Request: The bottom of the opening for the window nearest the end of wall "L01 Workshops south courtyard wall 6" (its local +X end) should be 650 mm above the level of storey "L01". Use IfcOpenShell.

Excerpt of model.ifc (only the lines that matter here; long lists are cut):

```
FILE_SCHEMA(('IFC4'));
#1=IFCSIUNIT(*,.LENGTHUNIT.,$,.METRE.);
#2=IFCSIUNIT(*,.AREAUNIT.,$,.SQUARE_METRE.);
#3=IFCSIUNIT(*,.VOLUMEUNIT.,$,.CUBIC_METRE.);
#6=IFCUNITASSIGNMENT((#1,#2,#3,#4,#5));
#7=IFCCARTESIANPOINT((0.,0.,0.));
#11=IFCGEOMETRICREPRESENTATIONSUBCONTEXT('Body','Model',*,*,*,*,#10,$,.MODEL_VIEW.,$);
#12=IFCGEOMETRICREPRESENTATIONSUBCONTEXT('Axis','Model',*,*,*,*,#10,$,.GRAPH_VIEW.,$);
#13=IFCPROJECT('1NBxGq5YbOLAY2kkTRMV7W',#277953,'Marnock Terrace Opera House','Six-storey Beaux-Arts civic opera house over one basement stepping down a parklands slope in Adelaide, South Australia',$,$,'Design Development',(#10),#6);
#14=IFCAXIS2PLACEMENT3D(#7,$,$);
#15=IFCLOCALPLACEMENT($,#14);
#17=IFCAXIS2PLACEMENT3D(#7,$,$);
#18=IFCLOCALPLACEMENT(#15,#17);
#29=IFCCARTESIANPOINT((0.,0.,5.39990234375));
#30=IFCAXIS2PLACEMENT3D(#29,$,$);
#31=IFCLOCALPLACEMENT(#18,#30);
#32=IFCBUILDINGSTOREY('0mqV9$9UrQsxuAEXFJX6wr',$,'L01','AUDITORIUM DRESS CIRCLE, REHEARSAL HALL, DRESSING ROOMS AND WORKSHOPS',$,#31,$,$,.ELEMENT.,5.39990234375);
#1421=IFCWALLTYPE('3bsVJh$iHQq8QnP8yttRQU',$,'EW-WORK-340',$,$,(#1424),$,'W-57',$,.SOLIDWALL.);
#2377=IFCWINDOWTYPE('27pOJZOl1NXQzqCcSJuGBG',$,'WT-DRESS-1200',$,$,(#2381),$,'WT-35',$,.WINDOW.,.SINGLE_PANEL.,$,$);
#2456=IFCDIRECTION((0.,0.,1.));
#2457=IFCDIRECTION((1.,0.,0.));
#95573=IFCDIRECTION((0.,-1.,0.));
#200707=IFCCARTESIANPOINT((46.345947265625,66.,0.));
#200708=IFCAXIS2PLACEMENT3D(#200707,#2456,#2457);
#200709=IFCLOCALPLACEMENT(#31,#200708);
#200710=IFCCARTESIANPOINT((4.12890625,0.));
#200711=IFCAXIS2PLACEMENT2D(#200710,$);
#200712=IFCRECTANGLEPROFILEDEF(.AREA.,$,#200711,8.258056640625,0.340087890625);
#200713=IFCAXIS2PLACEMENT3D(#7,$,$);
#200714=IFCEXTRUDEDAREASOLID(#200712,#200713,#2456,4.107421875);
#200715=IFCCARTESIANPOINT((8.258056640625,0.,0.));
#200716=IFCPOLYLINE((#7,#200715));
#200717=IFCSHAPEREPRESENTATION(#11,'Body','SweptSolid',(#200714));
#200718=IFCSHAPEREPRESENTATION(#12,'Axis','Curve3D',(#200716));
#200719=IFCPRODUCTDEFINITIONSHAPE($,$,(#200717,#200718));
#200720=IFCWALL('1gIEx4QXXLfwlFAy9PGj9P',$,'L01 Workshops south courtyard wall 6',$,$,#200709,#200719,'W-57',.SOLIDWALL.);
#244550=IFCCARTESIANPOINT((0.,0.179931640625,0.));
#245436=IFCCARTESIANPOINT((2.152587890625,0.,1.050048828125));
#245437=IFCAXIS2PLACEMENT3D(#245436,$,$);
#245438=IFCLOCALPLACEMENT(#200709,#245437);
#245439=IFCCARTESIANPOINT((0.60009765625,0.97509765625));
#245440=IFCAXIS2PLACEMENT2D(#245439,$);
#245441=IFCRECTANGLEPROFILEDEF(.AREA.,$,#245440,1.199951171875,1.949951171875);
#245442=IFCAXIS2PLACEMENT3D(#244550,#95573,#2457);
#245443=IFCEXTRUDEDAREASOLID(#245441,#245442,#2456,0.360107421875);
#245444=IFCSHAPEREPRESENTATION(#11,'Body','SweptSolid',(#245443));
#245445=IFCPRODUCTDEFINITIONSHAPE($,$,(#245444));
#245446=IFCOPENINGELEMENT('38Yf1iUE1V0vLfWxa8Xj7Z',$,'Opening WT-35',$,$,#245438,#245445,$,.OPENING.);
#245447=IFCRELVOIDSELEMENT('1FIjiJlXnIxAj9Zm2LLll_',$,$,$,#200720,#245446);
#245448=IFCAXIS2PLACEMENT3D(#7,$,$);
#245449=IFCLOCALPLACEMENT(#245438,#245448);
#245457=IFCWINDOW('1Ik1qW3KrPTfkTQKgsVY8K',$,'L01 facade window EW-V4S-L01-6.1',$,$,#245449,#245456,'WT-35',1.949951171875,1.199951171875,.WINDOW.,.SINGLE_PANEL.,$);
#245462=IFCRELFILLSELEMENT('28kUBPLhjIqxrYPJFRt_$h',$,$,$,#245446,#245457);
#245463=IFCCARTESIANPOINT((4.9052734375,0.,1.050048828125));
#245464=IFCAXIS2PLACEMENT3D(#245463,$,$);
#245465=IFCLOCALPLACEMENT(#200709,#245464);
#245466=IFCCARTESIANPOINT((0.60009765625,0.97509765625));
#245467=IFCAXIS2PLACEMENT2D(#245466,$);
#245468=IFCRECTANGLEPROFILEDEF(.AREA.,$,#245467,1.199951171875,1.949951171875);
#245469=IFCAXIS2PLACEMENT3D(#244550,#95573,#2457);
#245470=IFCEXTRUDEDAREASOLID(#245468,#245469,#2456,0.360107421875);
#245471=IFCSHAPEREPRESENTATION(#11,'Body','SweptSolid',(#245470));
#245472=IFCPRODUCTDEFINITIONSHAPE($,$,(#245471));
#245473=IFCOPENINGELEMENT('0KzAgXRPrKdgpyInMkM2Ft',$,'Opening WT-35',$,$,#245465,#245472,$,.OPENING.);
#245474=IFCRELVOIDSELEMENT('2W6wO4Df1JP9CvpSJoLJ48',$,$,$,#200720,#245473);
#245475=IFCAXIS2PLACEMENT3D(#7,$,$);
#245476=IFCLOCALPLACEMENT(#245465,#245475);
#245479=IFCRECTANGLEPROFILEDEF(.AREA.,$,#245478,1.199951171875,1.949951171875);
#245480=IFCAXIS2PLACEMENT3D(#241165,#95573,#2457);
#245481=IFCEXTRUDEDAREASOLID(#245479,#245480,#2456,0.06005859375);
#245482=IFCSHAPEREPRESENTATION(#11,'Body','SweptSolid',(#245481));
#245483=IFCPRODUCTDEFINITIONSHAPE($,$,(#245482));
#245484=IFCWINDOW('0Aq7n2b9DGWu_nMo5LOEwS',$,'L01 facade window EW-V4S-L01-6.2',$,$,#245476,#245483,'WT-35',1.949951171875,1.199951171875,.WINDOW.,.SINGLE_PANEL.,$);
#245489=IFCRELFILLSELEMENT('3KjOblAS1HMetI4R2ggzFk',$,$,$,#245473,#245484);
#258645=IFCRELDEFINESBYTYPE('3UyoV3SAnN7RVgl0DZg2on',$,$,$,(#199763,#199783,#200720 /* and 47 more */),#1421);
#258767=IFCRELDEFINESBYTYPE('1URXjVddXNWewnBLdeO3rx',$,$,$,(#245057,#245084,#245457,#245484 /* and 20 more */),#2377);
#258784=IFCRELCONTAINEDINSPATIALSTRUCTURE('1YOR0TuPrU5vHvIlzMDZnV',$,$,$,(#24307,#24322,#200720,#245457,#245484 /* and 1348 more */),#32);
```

```python
import numpy as np
import ifcopenshell
import ifcopenshell.api.geometry
import ifcopenshell.geom
import ifcopenshell.util.element
import ifcopenshell.util.placement
import ifcopenshell.util.shape
import ifcopenshell.util.unit

model = ifcopenshell.open("model.ifc")
unit_scale = ifcopenshell.util.unit.calculate_unit_scale(model)

window = model.by_guid("0Aq7n2b9DGWu_nMo5LOEwS")
opening = window.FillsVoids[0].RelatingOpeningElement
storey = ifcopenshell.util.element.get_container(window, ifc_class="IfcBuildingStorey")
level = ifcopenshell.util.placement.get_local_placement(storey.ObjectPlacement)[2, 3]

# The opening's origin need not be at the sill, so measure its lowest point.
shape = ifcopenshell.geom.create_shape(ifcopenshell.geom.settings(), opening)
bottom = ifcopenshell.util.shape.get_shape_bottom_elevation(shape, shape.geometry) / unit_scale
dz = level + 0.65 / unit_scale - bottom

shift = np.array([0.0, 0.0, dz])
# The window is placed relative to its opening, so it follows when the opening moves.
matrix = ifcopenshell.util.placement.get_local_placement(opening.ObjectPlacement)
matrix[:3, 3] += shift
ifcopenshell.api.geometry.edit_object_placement(
    model, product=opening, matrix=matrix, is_si=False, should_transform_children=True
)

print(f"moved by {dz * unit_scale:+.3f} m")

model.write("model-out.ifc")
```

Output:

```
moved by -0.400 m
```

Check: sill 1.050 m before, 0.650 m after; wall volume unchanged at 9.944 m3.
